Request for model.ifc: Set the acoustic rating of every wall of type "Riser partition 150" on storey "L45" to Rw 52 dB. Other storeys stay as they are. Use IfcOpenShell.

First a look at what the model holds.

```python
import ifcopenshell
import ifcopenshell.util.element

model = ifcopenshell.open("model.ifc")
print(model.schema)
storey = next(s for s in model.by_type("IfcBuildingStorey") if s.Name == "L45")
walls = [e for e in ifcopenshell.util.element.get_decomposition(storey) if e.is_a("IfcWall")]
seen = {}
for e in walls:
    element_type = ifcopenshell.util.element.get_type(e)
    key = (element_type.Name if element_type != e and element_type else None, ifcopenshell.util.element.get_pset(e, "Pset_WallCommon", "AcousticRating"))
    seen[key] = seen.get(key, 0) + 1
for (name, value), count in sorted(seen.items(), key=str):
    print(count, "x", name, "|", value)
```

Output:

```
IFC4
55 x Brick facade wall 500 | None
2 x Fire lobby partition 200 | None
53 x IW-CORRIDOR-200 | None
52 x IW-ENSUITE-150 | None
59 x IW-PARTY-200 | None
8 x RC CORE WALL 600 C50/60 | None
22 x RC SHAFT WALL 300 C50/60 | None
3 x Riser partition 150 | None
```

```python
import ifcopenshell
import ifcopenshell.api.pset
import ifcopenshell.util.element

model = ifcopenshell.open("model.ifc")

storey = next(s for s in model.by_type("IfcBuildingStorey") if s.Name == "L45")
walls = [e for e in ifcopenshell.util.element.get_decomposition(storey) if e.is_a("IfcWall")]

count = 0
for e in walls:
    element_type = ifcopenshell.util.element.get_type(e)
    if element_type in (None, e) or element_type.Name != "Riser partition 150":
        continue
    found = ifcopenshell.util.element.get_pset(e, "Pset_WallCommon", should_inherit=False)
    if found:
        pset = model.by_id(found["id"])
        if len(ifcopenshell.util.element.get_elements_by_pset(pset)) > 1:
            pset = ifcopenshell.api.pset.unshare_pset(model, products=[e], pset=pset)[0]
    else:
        pset = ifcopenshell.api.pset.add_pset(model, product=e, name="Pset_WallCommon")
    ifcopenshell.api.pset.edit_pset(model, pset=pset, properties={"AcousticRating": "Rw 52 dB"})
    count += 1

print(count, "walls updated")

model.write("model_rev.ifc")
```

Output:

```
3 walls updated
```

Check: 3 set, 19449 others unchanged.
